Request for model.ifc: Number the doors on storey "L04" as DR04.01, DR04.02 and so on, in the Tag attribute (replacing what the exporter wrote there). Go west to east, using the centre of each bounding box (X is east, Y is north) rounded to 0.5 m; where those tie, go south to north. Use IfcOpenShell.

First a look at what the model holds.

```python
import ifcopenshell
import ifcopenshell.util.element
import ifcopenshell.util.placement

model = ifcopenshell.open("model.ifc")
print(model.schema)
storey = next(s for s in model.by_type("IfcBuildingStorey") if s.Name == "L04")
doors = [e for e in ifcopenshell.util.element.get_decomposition(storey) if e.is_a("IfcDoor")]
for e in sorted(doors, key=lambda e: e.id()):
    origin = ifcopenshell.util.placement.get_local_placement(e.ObjectPlacement)[:3, 3]
    print(e.id(), e.Tag, e.Name, origin.round(2) + 0.0, sep=" | ")
```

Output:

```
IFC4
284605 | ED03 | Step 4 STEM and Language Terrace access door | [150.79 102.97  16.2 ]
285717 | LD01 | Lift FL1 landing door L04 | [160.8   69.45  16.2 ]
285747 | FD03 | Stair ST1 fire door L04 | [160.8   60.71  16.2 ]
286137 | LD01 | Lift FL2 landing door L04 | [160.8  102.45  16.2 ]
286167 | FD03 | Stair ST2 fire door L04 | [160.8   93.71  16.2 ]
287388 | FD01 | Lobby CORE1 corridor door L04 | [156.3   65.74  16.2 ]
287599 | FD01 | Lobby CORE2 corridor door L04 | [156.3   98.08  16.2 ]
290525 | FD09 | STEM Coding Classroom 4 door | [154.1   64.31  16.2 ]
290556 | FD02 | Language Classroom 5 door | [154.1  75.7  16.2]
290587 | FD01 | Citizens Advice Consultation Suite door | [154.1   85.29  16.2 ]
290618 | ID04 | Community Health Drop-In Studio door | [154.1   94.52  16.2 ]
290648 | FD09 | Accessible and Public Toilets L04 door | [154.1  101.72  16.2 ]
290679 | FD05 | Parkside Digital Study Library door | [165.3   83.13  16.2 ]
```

```python
import ifcopenshell
import ifcopenshell.geom
import ifcopenshell.util.element
import ifcopenshell.util.shape

model = ifcopenshell.open("model.ifc")
settings = ifcopenshell.geom.settings()
settings.set("use-world-coords", True)


def centre(element):
    shape = ifcopenshell.geom.create_shape(settings, element)
    return ifcopenshell.util.shape.get_bbox_centroid(shape.geometry)


storey = next(s for s in model.by_type("IfcBuildingStorey") if s.Name == "L04")
doors = [e for e in ifcopenshell.util.element.get_decomposition(storey) if e.is_a("IfcDoor")]

# Insertion points can sit at a corner or the storey origin, so sort by the geometry (in metres).
centres = {e: centre(e) for e in doors}
doors.sort(key=lambda e: (round(centres[e][0] / 0.5), centres[e][1]))

for i, e in enumerate(doors, start=1):
    number = f"DR04.{i:02d}"
    e.Tag = number
    print(e.id(), number)

model.write("model_rev.ifc")
```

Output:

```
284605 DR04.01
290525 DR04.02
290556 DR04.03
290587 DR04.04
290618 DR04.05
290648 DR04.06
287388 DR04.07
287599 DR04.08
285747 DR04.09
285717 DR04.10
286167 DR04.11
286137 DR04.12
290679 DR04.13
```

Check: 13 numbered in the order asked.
